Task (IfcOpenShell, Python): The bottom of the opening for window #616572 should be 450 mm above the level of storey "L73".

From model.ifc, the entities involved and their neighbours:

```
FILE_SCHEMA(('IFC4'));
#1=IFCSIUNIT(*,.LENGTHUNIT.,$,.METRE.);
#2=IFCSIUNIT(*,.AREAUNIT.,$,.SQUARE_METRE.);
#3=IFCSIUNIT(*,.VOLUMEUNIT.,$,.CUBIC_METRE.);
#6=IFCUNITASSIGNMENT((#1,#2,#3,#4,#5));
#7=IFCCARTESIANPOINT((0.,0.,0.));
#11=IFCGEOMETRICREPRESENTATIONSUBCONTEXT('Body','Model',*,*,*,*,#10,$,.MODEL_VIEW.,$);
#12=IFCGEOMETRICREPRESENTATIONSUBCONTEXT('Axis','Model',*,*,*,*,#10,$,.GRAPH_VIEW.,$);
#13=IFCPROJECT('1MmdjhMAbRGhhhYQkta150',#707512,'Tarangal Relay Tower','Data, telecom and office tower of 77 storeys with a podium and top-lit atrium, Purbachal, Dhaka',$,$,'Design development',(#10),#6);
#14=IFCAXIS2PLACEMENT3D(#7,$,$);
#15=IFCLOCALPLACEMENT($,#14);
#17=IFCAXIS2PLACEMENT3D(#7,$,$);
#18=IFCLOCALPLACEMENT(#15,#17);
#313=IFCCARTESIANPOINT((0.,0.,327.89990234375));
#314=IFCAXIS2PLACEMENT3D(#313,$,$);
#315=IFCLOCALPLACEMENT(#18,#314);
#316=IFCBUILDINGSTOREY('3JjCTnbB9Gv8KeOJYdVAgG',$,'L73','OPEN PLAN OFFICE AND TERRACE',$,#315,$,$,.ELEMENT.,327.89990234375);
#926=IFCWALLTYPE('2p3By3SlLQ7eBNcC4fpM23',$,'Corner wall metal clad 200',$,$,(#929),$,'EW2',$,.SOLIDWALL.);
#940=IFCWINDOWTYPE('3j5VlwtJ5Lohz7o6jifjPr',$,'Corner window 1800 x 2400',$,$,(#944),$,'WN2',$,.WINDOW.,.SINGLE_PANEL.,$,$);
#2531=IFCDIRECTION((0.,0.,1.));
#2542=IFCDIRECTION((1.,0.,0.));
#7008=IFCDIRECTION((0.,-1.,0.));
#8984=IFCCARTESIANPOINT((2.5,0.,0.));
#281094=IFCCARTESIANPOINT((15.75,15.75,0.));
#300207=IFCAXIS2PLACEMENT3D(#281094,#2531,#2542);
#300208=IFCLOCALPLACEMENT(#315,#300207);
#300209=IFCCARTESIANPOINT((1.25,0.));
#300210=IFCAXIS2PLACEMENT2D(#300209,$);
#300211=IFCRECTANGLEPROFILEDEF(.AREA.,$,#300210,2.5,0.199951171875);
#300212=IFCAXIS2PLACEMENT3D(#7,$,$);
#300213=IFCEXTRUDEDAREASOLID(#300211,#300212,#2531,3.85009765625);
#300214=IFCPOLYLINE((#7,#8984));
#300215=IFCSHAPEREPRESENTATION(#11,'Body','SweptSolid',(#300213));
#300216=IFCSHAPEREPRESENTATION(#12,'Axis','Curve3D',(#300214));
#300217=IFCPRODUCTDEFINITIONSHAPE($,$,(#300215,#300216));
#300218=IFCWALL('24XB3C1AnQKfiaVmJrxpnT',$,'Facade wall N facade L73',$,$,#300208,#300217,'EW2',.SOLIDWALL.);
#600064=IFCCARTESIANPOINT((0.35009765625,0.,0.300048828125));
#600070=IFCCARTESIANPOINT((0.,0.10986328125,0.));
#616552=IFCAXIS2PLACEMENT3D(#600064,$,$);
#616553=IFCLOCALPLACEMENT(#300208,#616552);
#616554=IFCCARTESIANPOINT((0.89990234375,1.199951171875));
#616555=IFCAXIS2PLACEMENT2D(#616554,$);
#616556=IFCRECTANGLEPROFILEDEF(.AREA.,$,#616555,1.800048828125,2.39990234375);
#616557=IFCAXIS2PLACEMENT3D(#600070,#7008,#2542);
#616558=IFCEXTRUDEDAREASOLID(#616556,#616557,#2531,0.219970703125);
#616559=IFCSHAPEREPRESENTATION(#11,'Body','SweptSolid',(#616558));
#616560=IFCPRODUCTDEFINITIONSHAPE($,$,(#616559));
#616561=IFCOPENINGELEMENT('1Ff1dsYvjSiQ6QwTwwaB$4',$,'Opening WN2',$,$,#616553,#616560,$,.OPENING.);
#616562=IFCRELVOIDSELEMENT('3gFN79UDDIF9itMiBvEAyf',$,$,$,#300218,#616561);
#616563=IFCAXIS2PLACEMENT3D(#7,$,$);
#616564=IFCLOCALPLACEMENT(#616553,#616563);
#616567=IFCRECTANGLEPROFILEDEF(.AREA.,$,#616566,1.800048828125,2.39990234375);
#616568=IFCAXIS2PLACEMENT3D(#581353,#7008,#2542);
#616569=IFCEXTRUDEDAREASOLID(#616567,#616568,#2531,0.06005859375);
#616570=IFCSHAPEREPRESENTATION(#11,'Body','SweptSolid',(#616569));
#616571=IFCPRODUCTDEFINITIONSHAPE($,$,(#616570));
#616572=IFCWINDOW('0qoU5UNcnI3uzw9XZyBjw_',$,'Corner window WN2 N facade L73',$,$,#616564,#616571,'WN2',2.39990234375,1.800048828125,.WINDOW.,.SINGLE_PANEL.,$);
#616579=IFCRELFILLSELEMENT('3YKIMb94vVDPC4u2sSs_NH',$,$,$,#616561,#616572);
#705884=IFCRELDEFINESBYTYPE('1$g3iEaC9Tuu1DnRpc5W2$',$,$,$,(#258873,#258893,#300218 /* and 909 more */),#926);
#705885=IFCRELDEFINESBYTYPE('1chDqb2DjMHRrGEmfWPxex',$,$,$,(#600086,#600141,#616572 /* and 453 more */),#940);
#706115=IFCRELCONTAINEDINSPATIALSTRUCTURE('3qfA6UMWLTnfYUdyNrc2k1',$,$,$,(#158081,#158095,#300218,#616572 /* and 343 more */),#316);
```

```python
import numpy as np
import ifcopenshell
import ifcopenshell.api.geometry
import ifcopenshell.geom
import ifcopenshell.util.element
import ifcopenshell.util.placement
import ifcopenshell.util.shape
import ifcopenshell.util.unit

model = ifcopenshell.open("model.ifc")
unit_scale = ifcopenshell.util.unit.calculate_unit_scale(model)

window = model.by_guid("0qoU5UNcnI3uzw9XZyBjw_")
opening = window.FillsVoids[0].RelatingOpeningElement
storey = ifcopenshell.util.element.get_container(window, ifc_class="IfcBuildingStorey")
level = ifcopenshell.util.placement.get_local_placement(storey.ObjectPlacement)[2, 3]

# The opening's origin need not be at the sill, so measure its lowest point.
shape = ifcopenshell.geom.create_shape(ifcopenshell.geom.settings(), opening)
bottom = ifcopenshell.util.shape.get_shape_bottom_elevation(shape, shape.geometry) / unit_scale
dz = level + 0.45 / unit_scale - bottom

shift = np.array([0.0, 0.0, dz])
# The window is placed relative to its opening, so it follows when the opening moves.
matrix = ifcopenshell.util.placement.get_local_placement(opening.ObjectPlacement)
matrix[:3, 3] += shift
ifcopenshell.api.geometry.edit_object_placement(
    model, product=opening, matrix=matrix, is_si=False, should_transform_children=True
)

print(f"moved by {dz * unit_scale:+.3f} m")

model.write("model_updated.ifc")
```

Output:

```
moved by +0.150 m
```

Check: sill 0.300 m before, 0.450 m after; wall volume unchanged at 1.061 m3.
